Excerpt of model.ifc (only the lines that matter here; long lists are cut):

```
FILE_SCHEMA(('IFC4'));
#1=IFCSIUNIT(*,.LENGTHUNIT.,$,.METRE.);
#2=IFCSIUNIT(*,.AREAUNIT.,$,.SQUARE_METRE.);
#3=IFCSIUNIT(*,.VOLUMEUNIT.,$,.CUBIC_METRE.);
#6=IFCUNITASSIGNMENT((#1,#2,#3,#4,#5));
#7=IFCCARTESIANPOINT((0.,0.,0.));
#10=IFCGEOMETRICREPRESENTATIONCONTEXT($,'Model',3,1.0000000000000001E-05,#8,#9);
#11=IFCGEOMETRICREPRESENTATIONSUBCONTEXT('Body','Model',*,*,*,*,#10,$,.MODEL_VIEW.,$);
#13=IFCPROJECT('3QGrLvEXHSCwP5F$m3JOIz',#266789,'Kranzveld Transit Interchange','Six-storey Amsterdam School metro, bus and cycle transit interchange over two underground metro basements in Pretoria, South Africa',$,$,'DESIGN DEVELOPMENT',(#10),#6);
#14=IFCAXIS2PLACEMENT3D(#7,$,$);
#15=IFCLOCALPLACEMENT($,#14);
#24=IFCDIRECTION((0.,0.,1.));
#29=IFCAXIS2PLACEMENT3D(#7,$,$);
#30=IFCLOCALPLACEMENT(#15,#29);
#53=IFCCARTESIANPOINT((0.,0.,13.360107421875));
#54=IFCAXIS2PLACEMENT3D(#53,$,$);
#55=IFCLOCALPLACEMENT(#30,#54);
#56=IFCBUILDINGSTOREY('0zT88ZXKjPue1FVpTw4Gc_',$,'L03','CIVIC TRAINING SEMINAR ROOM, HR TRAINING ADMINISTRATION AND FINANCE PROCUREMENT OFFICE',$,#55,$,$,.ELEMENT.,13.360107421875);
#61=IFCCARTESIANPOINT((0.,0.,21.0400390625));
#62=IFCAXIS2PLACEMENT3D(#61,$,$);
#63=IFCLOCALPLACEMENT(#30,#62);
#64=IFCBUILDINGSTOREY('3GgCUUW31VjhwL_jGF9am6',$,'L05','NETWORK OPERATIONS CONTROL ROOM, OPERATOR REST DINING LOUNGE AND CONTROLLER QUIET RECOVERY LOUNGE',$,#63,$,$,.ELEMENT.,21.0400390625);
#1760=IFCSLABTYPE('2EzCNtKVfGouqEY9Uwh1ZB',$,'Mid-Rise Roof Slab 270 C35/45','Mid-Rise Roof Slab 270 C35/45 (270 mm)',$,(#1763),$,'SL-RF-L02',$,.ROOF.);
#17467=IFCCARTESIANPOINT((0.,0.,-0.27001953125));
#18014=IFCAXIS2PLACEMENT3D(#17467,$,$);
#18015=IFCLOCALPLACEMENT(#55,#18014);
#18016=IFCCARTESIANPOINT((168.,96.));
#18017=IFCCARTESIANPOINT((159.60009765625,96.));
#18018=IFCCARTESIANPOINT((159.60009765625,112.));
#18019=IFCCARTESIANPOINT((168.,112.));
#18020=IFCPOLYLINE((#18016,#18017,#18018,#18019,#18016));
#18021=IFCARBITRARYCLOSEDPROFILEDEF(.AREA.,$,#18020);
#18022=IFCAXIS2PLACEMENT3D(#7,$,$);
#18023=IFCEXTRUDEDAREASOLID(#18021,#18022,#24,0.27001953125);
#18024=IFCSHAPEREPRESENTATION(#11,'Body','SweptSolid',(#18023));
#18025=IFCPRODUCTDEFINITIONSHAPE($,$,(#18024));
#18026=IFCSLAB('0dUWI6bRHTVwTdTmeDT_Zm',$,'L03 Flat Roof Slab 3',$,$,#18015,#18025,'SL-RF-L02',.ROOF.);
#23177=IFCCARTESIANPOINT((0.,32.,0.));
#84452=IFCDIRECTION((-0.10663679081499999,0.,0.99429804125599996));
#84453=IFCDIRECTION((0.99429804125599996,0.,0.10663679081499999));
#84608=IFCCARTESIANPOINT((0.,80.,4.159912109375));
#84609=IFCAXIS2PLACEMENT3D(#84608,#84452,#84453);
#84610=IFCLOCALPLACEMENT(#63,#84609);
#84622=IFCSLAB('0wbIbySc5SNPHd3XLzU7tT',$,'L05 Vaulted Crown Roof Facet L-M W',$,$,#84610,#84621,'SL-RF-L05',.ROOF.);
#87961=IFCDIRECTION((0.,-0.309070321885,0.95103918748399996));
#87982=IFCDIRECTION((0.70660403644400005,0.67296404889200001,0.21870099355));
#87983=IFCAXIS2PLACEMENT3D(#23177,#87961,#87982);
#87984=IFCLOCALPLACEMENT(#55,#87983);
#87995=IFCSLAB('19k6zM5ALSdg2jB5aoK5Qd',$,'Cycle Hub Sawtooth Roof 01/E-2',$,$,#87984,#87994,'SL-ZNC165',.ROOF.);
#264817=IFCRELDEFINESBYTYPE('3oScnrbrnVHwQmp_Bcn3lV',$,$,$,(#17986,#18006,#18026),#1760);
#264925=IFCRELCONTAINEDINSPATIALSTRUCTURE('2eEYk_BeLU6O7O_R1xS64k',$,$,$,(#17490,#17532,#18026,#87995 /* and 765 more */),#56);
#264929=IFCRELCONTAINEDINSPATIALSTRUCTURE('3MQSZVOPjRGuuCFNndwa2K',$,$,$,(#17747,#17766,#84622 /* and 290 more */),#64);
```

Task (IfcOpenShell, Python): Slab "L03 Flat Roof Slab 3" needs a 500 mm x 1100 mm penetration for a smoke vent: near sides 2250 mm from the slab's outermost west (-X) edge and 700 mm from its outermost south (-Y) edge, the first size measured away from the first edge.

```python
import numpy as np
import ifcopenshell
import ifcopenshell.api.feature
import ifcopenshell.api.geometry
import ifcopenshell.api.root
import ifcopenshell.geom
import ifcopenshell.util.placement
import ifcopenshell.util.representation
import ifcopenshell.util.shape
import ifcopenshell.util.unit

model = ifcopenshell.open("model.ifc")
unit_scale = ifcopenshell.util.unit.calculate_unit_scale(model)
settings = ifcopenshell.geom.settings()


def volume(element):
    """Net volume in cubic metres, openings subtracted."""
    shape = ifcopenshell.geom.create_shape(settings, element)
    return ifcopenshell.util.shape.get_volume(shape.geometry)


slab = model.by_id(18026)
before = volume(slab)

# Extent in the slab's own axes, in metres. The edges named are its -X and -Y sides.
slab_shape = ifcopenshell.geom.create_shape(settings, slab)
vertices = ifcopenshell.util.shape.get_vertices(slab_shape.geometry)
x_min, y_min, bottom = vertices.min(axis=0)
top = vertices[:, 2].max()

opening = ifcopenshell.api.root.create_entity(model, ifc_class="IfcOpeningElement", name="Smoke vent opening", predefined_type="OPENING")
context = ifcopenshell.util.representation.get_context(model, "Model", "Body", "MODEL_VIEW")
width, depth = 0.5, 1.1
outline = [(0.0, 0.0), (width, 0.0), (width, depth), (0.0, depth), (0.0, 0.0)]
# Overshoot both faces by 50 mm so the cut is clean.
shape = ifcopenshell.api.geometry.add_slab_representation(
    model, context=context, depth=top - bottom + 0.1, polyline=outline
)
ifcopenshell.api.geometry.assign_representation(model, product=opening, representation=shape)

matrix = ifcopenshell.util.placement.get_local_placement(slab.ObjectPlacement)
matrix[:, 3] = matrix @ np.append(np.array([x_min + 2.25, y_min + 0.7, bottom - 0.05]) / unit_scale, 1.0)
ifcopenshell.api.geometry.edit_object_placement(model, product=opening, matrix=matrix, is_si=False)
ifcopenshell.api.feature.add_feature(model, feature=opening, element=slab)

after = volume(slab)

print(f"slab volume {before:.3f} -> {after:.3f} m3")

model.write("model_v2.ifc")
```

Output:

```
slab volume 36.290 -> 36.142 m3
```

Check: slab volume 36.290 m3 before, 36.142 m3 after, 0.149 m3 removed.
